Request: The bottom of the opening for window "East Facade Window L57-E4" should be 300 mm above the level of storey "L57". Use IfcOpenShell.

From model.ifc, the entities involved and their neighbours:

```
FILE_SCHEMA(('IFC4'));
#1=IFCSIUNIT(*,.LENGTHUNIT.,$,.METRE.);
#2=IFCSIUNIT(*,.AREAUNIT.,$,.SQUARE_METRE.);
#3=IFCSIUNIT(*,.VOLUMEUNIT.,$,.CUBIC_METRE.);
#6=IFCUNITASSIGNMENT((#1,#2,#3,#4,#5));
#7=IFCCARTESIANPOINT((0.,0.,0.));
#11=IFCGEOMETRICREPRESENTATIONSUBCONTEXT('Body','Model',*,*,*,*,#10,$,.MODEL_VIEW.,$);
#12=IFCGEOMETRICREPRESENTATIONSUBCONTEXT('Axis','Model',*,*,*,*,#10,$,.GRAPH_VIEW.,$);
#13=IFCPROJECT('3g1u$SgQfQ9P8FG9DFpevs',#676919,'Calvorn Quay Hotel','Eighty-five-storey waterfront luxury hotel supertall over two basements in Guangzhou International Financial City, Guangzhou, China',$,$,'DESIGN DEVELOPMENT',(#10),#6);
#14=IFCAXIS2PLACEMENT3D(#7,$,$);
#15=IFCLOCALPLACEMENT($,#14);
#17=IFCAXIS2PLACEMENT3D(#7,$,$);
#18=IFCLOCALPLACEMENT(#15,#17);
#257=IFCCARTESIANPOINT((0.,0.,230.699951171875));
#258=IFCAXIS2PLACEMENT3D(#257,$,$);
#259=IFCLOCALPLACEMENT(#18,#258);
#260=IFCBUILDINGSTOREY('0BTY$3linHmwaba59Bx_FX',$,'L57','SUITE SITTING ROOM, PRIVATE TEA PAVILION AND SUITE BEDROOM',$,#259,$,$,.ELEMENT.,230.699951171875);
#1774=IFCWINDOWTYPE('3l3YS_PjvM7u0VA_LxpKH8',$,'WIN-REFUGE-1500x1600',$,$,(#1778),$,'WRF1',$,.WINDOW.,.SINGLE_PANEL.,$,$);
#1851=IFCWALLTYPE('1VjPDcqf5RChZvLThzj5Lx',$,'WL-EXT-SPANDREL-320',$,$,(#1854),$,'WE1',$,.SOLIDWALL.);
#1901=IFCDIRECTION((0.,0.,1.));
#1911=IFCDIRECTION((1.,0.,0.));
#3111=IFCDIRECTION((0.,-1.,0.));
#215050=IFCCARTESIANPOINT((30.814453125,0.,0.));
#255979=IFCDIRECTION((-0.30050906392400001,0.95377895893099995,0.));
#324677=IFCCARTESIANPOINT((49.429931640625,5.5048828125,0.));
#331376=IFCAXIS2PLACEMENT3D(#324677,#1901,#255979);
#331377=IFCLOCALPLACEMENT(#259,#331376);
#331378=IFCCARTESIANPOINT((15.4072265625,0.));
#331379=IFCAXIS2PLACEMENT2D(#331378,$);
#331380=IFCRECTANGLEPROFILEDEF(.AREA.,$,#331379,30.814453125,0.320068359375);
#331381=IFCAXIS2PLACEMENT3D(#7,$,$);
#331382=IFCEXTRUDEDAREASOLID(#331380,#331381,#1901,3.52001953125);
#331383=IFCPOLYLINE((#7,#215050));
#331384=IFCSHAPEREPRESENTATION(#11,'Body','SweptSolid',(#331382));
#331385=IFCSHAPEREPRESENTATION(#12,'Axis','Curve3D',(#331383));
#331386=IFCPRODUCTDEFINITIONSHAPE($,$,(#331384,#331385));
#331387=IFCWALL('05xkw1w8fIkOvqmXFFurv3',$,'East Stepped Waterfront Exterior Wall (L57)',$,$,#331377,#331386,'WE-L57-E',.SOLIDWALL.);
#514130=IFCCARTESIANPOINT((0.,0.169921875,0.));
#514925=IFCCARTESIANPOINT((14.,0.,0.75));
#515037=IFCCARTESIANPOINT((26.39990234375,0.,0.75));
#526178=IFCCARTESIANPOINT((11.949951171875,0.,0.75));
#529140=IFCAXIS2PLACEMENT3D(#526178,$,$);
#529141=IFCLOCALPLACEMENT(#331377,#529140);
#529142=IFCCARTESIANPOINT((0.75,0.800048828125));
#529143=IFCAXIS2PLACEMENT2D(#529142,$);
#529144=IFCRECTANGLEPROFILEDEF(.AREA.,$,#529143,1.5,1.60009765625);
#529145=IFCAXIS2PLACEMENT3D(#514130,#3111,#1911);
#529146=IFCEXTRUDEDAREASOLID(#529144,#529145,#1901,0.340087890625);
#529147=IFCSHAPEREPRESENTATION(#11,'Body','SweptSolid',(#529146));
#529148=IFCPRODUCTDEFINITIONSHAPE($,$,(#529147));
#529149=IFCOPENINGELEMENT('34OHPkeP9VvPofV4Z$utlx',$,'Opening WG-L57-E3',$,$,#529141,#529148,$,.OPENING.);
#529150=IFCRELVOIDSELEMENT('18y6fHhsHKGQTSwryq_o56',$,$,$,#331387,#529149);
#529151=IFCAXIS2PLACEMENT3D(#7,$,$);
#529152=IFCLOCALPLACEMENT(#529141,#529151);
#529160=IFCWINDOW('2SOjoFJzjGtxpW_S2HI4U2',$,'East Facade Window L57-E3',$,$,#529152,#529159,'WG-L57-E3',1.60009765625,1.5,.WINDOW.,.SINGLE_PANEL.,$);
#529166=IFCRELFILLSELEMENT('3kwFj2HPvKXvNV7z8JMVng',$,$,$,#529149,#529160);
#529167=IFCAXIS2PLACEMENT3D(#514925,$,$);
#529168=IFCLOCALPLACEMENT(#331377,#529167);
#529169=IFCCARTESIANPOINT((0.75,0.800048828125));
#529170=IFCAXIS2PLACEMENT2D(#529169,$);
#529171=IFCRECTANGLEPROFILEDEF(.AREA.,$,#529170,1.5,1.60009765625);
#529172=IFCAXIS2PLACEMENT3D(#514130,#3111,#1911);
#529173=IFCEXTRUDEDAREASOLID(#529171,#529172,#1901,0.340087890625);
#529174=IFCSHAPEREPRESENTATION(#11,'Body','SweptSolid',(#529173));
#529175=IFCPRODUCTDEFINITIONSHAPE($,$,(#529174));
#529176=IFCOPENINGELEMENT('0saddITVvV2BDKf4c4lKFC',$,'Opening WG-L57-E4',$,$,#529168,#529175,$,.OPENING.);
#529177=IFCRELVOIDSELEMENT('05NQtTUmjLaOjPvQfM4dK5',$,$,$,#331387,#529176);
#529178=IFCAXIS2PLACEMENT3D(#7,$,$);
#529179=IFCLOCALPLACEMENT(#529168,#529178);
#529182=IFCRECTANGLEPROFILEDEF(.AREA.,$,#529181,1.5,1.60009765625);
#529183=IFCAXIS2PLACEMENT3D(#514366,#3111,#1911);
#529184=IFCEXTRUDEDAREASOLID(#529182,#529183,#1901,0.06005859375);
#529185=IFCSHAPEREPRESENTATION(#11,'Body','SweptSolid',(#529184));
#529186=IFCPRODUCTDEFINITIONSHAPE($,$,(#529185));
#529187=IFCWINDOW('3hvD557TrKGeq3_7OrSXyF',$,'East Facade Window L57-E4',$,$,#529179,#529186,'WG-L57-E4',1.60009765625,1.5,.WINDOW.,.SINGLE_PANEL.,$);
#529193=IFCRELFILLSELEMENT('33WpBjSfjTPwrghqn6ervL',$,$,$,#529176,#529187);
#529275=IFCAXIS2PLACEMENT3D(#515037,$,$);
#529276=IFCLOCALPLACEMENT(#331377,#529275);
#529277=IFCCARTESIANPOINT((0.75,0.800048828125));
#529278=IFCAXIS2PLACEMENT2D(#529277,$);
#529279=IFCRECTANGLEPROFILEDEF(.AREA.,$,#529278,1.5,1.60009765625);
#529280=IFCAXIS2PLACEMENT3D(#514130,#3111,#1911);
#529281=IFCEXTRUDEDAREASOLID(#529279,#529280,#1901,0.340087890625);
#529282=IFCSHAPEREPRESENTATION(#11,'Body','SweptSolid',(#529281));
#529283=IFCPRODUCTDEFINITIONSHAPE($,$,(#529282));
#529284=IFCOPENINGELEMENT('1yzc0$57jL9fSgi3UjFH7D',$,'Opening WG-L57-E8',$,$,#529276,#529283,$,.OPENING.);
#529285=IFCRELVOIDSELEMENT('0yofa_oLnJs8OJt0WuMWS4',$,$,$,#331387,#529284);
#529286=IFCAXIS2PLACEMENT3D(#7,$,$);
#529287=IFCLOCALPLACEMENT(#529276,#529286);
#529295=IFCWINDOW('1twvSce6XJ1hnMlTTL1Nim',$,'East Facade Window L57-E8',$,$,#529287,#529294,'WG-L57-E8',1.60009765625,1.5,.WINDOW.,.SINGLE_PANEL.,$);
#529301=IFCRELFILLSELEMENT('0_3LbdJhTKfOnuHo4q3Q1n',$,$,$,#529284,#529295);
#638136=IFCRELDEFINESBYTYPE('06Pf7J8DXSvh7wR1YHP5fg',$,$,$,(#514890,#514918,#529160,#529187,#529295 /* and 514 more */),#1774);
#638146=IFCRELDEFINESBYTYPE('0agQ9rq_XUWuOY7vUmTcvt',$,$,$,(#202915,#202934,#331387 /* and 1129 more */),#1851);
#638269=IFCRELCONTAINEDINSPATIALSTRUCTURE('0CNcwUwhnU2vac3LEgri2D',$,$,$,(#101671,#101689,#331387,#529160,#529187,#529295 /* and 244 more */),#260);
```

```python
import numpy as np
import ifcopenshell
import ifcopenshell.api.geometry
import ifcopenshell.geom
import ifcopenshell.util.element
import ifcopenshell.util.placement
import ifcopenshell.util.shape
import ifcopenshell.util.unit

model = ifcopenshell.open("model.ifc")
unit_scale = ifcopenshell.util.unit.calculate_unit_scale(model)

window = model.by_guid("3hvD557TrKGeq3_7OrSXyF")
opening = window.FillsVoids[0].RelatingOpeningElement
storey = ifcopenshell.util.element.get_container(window, ifc_class="IfcBuildingStorey")
level = ifcopenshell.util.placement.get_local_placement(storey.ObjectPlacement)[2, 3]

# The opening's origin need not be at the sill, so measure its lowest point.
shape = ifcopenshell.geom.create_shape(ifcopenshell.geom.settings(), opening)
bottom = ifcopenshell.util.shape.get_shape_bottom_elevation(shape, shape.geometry) / unit_scale
dz = level + 0.3 / unit_scale - bottom

shift = np.array([0.0, 0.0, dz])
# The window is placed relative to its opening, so it follows when the opening moves.
matrix = ifcopenshell.util.placement.get_local_placement(opening.ObjectPlacement)
matrix[:3, 3] += shift
ifcopenshell.api.geometry.edit_object_placement(
    model, product=opening, matrix=matrix, is_si=False, should_transform_children=True
)

print(f"moved by {dz * unit_scale:+.3f} m")

model.write("model_edited.ifc")
```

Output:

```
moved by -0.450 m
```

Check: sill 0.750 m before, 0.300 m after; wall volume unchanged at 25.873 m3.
